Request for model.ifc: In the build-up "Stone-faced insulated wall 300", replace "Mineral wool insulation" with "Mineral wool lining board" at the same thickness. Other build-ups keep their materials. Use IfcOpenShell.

First a look at what the model holds.

```python
import ifcopenshell
import ifcopenshell.util.element

model = ifcopenshell.open("model.ifc")
print(model.schema)
for layer_set in model.by_type("IfcMaterialLayerSet"):
    if layer_set.LayerSetName == "Stone-faced insulated wall 300":
        for layer in layer_set.MaterialLayers:
            print(layer.id(), layer.Material and layer.Material.Name, layer.LayerThickness, sep=" | ")
        print(len(ifcopenshell.util.element.get_elements_by_material(model, layer_set)), "elements and types use it")
print(sorted(m.Name for m in model.by_type("IfcMaterial") if m.Name)[:60])
```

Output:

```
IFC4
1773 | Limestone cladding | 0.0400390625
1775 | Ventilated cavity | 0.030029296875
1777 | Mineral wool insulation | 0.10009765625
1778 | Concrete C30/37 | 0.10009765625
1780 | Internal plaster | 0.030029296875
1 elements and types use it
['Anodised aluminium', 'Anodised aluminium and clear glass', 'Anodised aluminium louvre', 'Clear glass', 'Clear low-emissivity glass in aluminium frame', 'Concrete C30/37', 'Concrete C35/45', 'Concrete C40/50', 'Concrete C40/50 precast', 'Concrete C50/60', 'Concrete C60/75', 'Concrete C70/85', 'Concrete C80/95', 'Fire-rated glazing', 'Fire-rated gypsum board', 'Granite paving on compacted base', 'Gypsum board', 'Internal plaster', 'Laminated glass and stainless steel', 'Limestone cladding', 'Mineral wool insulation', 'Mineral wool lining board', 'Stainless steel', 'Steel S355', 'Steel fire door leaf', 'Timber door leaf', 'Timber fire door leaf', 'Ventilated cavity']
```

```python
import ifcopenshell
import ifcopenshell.api.material

model = ifcopenshell.open("model.ifc")

layer_set = next(s for s in model.by_type("IfcMaterialLayerSet") if s.LayerSetName == "Stone-faced insulated wall 300")
layer = next(l for l in layer_set.MaterialLayers if l.Material and l.Material.Name == "Mineral wool insulation")
material = next(m for m in model.by_type("IfcMaterial") if m.Name == "Mineral wool lining board")

# Point this one layer at the other material; renaming the old one would change it everywhere.
ifcopenshell.api.material.edit_layer(model, layer=layer, attributes={}, material=material)

print([l.Material.Name if l.Material else None for l in layer_set.MaterialLayers])

model.write("model_updated.ifc")
```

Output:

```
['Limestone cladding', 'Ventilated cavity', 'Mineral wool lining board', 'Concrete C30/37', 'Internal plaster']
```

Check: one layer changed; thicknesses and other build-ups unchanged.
